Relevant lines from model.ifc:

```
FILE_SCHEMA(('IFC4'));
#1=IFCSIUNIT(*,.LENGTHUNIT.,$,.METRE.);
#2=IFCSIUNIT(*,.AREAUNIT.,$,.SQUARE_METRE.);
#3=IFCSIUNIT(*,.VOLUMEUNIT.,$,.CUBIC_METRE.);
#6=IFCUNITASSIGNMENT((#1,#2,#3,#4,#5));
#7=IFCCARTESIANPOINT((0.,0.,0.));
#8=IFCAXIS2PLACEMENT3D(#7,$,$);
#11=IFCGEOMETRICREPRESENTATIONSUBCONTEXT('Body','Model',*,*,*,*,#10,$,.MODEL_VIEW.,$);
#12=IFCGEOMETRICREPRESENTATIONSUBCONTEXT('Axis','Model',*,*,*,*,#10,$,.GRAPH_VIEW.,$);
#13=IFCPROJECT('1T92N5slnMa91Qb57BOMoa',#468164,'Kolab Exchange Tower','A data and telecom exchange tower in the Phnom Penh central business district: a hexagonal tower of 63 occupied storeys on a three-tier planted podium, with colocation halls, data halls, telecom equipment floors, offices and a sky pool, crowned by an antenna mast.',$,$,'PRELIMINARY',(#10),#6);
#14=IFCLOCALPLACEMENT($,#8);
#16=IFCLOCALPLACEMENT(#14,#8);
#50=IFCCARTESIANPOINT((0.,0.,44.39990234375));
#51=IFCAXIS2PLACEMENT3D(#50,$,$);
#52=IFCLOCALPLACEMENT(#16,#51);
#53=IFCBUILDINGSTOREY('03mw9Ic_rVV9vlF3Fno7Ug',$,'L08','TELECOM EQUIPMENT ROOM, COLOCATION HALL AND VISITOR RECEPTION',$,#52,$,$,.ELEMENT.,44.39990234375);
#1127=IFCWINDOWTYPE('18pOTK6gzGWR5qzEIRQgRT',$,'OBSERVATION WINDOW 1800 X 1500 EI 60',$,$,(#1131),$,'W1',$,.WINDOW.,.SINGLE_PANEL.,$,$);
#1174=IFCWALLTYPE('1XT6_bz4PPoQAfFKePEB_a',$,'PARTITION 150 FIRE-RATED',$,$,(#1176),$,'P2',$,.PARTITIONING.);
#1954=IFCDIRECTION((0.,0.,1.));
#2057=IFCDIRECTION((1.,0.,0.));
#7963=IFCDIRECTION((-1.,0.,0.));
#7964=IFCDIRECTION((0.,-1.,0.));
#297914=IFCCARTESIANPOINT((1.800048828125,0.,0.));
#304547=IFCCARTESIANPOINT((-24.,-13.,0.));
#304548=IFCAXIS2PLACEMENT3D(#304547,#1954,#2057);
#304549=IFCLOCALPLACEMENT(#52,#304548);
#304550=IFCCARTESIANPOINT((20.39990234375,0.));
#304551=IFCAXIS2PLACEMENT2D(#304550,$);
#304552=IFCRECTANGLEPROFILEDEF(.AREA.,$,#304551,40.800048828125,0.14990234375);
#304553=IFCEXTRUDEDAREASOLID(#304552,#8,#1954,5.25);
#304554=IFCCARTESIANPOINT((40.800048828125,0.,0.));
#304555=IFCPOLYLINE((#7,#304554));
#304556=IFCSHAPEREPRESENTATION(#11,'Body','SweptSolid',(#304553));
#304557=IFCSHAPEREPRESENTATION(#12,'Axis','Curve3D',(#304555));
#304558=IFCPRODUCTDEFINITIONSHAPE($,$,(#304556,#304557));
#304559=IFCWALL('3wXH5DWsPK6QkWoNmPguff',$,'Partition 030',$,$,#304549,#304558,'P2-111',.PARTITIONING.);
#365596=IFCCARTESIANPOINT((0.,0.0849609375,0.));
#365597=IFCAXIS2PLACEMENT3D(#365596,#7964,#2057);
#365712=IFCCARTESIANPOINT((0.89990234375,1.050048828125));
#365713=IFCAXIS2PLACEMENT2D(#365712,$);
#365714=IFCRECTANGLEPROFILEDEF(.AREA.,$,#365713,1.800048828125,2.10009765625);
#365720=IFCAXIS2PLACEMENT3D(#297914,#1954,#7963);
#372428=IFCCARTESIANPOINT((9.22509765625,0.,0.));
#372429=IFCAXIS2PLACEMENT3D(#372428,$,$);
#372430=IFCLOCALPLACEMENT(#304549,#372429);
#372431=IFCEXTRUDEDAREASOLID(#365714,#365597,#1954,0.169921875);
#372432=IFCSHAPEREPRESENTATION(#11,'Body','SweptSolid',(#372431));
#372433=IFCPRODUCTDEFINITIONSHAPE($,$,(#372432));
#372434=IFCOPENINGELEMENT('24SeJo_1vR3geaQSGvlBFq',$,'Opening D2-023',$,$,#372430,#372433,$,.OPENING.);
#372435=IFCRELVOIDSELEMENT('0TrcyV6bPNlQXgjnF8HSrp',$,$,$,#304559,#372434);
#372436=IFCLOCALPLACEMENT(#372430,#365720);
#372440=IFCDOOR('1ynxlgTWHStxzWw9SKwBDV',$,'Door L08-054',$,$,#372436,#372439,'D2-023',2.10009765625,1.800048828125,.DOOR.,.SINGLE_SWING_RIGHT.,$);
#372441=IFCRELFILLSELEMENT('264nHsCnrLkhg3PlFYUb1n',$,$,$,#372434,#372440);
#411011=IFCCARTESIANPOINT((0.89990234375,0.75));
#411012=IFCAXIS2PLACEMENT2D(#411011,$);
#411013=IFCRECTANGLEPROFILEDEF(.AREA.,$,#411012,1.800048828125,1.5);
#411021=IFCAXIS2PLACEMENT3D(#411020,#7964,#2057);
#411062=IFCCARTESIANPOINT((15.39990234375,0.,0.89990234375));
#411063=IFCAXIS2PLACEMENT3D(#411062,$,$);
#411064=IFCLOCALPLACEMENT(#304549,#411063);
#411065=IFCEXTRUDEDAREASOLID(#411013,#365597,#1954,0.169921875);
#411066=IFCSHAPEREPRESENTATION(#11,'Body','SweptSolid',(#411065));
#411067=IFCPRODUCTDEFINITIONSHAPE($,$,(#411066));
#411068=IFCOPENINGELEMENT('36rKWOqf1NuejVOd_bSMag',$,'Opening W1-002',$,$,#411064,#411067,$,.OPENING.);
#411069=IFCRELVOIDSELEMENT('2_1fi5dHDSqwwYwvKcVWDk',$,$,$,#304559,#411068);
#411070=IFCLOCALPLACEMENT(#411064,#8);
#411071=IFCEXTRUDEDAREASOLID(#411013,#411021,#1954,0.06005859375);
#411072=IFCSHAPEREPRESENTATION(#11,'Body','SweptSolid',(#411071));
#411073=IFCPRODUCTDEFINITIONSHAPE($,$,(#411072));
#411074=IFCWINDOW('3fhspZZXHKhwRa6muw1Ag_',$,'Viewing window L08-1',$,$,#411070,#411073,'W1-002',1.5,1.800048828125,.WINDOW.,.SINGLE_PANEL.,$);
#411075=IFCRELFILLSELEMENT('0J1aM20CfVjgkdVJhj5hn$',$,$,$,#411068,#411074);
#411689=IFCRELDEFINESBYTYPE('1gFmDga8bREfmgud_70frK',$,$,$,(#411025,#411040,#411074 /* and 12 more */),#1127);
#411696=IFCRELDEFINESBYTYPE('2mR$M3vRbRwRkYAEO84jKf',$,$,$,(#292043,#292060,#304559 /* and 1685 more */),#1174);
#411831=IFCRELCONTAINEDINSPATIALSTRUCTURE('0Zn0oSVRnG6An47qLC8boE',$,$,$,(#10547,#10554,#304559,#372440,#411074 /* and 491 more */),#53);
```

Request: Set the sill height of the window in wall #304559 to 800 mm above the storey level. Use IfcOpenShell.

```python
import numpy as np
import ifcopenshell
import ifcopenshell.api.geometry
import ifcopenshell.geom
import ifcopenshell.util.element
import ifcopenshell.util.placement
import ifcopenshell.util.shape
import ifcopenshell.util.unit

model = ifcopenshell.open("model.ifc")
unit_scale = ifcopenshell.util.unit.calculate_unit_scale(model)

window = model.by_guid("3fhspZZXHKhwRa6muw1Ag_")
opening = window.FillsVoids[0].RelatingOpeningElement
storey = ifcopenshell.util.element.get_container(window, ifc_class="IfcBuildingStorey")
level = ifcopenshell.util.placement.get_local_placement(storey.ObjectPlacement)[2, 3]

# The opening's origin need not be at the sill, so measure its lowest point.
shape = ifcopenshell.geom.create_shape(ifcopenshell.geom.settings(), opening)
bottom = ifcopenshell.util.shape.get_shape_bottom_elevation(shape, shape.geometry) / unit_scale
dz = level + 0.8 / unit_scale - bottom

shift = np.array([0.0, 0.0, dz])
# The window is placed relative to its opening, so it follows when the opening moves.
matrix = ifcopenshell.util.placement.get_local_placement(opening.ObjectPlacement)
matrix[:3, 3] += shift
ifcopenshell.api.geometry.edit_object_placement(
    model, product=opening, matrix=matrix, is_si=False, should_transform_children=True
)

print(f"moved by {dz * unit_scale:+.3f} m")

model.write("model_updated.ifc")
```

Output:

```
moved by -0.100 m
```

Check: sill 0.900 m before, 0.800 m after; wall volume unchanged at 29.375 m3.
